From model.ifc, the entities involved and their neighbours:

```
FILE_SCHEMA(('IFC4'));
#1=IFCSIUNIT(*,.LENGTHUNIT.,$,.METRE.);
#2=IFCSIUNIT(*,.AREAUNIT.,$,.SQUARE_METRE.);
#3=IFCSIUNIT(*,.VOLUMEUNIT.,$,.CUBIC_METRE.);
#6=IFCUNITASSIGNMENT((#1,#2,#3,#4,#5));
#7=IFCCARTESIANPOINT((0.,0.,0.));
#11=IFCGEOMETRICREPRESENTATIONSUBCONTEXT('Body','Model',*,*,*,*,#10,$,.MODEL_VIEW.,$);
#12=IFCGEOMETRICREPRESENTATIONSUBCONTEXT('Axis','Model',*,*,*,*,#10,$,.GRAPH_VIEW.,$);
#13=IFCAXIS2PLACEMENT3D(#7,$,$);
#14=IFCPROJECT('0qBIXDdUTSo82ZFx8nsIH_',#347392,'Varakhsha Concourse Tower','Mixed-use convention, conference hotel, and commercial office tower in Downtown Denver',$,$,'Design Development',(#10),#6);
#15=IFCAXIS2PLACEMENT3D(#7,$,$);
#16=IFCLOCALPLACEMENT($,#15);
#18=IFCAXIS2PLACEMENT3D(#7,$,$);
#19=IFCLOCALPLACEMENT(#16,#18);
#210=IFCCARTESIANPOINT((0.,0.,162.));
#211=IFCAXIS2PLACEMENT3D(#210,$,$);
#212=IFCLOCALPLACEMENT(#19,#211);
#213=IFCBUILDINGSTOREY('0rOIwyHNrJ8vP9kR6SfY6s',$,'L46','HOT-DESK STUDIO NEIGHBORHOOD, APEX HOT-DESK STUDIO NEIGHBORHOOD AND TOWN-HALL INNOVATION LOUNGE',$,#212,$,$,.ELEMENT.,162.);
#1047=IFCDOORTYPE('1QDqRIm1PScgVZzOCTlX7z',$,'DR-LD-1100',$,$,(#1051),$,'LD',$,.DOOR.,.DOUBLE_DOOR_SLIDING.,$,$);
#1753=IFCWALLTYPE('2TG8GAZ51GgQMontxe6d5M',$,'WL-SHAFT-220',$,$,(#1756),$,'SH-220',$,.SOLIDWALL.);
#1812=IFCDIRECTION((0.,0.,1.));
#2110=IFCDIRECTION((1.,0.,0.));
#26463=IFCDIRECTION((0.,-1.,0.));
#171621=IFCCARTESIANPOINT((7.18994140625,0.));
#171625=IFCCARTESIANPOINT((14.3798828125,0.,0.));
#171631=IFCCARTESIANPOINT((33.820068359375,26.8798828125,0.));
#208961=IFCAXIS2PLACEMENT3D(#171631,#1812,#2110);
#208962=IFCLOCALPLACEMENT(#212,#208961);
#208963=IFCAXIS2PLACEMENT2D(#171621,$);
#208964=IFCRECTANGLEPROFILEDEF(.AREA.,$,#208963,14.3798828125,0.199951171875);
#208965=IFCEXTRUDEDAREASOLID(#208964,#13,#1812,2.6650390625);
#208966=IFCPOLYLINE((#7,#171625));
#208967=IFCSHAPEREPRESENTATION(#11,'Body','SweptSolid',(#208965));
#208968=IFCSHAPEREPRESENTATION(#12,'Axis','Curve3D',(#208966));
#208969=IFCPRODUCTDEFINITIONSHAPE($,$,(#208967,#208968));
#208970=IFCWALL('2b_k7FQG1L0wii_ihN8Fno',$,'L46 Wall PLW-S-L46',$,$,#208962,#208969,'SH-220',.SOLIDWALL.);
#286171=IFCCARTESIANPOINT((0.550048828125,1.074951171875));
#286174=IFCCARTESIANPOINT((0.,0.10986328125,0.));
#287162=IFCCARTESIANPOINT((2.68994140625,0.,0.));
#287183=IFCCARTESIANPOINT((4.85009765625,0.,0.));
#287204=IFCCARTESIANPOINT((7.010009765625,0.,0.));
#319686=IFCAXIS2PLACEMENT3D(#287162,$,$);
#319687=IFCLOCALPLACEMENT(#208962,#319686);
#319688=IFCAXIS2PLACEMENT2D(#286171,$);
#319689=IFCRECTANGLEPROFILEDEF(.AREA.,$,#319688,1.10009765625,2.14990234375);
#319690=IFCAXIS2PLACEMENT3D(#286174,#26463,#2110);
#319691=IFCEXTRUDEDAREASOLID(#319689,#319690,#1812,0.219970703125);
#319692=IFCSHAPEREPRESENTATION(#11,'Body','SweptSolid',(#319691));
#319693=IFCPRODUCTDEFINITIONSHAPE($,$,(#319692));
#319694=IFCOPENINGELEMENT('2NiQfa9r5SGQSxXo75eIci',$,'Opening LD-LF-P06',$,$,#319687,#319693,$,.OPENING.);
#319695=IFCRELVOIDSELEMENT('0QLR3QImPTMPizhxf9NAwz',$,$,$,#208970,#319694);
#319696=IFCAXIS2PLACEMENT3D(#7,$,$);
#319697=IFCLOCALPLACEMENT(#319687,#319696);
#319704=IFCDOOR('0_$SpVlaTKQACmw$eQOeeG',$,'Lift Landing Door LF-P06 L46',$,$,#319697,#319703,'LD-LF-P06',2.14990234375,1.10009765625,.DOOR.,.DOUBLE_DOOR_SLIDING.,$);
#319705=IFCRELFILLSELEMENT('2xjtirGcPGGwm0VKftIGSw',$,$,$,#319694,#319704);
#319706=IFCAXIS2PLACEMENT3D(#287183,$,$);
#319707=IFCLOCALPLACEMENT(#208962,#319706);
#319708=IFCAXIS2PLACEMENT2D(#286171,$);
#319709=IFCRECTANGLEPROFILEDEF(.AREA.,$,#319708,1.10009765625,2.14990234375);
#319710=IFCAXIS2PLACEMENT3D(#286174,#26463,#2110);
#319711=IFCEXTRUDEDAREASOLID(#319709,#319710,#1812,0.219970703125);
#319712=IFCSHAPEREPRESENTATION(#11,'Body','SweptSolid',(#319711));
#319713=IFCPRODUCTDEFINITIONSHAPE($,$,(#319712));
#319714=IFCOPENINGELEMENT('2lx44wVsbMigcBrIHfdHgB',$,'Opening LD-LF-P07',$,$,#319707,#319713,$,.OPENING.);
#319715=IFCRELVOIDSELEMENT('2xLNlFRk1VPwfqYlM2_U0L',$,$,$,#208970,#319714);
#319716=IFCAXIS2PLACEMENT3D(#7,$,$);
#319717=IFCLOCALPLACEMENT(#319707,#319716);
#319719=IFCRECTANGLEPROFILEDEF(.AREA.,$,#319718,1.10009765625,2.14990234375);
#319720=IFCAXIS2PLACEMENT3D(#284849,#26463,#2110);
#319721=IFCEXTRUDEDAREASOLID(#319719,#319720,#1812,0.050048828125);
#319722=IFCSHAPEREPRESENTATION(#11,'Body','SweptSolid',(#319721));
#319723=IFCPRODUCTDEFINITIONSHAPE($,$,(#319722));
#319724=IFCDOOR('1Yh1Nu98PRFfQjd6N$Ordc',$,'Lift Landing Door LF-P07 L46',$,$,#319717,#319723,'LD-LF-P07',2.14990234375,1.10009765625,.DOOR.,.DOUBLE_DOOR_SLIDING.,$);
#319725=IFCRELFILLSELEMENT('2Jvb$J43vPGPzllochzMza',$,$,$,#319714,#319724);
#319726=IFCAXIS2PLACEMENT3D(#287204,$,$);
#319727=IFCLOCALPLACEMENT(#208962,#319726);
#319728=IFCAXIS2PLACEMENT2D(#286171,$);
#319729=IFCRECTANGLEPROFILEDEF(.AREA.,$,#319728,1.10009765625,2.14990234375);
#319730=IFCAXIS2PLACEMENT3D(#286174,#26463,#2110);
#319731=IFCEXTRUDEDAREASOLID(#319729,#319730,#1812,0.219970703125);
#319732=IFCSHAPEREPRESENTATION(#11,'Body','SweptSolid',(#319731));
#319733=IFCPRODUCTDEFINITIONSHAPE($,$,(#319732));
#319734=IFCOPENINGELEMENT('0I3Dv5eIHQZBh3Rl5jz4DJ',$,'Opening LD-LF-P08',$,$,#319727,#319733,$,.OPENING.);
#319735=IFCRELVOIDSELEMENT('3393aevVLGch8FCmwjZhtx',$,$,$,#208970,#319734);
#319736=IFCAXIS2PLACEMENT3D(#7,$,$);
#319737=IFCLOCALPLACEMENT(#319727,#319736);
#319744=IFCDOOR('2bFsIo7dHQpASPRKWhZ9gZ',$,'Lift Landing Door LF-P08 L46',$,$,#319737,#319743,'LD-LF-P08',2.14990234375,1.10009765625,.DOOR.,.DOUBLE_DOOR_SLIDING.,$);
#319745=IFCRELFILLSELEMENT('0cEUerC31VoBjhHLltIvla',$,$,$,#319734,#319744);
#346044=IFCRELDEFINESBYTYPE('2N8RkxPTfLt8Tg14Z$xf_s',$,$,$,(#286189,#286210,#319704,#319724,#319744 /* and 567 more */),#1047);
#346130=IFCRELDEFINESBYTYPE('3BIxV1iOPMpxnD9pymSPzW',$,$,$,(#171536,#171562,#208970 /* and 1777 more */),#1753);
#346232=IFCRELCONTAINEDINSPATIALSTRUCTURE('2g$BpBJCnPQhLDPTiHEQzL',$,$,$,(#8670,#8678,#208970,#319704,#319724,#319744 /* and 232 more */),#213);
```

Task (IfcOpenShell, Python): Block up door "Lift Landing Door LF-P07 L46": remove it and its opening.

```python
import ifcopenshell
import ifcopenshell.api.feature
import ifcopenshell.api.root
import ifcopenshell.geom
import ifcopenshell.util.shape

model = ifcopenshell.open("model.ifc")
settings = ifcopenshell.geom.settings()


def volume(element):
    """Net volume in cubic metres, openings subtracted."""
    shape = ifcopenshell.geom.create_shape(settings, element)
    return ifcopenshell.util.shape.get_volume(shape.geometry)


door = model.by_guid("1Yh1Nu98PRFfQjd6N$Ordc")
opening = door.FillsVoids[0].RelatingOpeningElement
wall = opening.VoidsElements[0].RelatingBuildingElement
before = volume(wall)

ifcopenshell.api.root.remove_product(model, product=door)
ifcopenshell.api.feature.remove_feature(model, feature=opening)

after = volume(wall)

print(f"wall volume {before:.3f} -> {after:.3f} m3")

model.write("model-out.ifc")
```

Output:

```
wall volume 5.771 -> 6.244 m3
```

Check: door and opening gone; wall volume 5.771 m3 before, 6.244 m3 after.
